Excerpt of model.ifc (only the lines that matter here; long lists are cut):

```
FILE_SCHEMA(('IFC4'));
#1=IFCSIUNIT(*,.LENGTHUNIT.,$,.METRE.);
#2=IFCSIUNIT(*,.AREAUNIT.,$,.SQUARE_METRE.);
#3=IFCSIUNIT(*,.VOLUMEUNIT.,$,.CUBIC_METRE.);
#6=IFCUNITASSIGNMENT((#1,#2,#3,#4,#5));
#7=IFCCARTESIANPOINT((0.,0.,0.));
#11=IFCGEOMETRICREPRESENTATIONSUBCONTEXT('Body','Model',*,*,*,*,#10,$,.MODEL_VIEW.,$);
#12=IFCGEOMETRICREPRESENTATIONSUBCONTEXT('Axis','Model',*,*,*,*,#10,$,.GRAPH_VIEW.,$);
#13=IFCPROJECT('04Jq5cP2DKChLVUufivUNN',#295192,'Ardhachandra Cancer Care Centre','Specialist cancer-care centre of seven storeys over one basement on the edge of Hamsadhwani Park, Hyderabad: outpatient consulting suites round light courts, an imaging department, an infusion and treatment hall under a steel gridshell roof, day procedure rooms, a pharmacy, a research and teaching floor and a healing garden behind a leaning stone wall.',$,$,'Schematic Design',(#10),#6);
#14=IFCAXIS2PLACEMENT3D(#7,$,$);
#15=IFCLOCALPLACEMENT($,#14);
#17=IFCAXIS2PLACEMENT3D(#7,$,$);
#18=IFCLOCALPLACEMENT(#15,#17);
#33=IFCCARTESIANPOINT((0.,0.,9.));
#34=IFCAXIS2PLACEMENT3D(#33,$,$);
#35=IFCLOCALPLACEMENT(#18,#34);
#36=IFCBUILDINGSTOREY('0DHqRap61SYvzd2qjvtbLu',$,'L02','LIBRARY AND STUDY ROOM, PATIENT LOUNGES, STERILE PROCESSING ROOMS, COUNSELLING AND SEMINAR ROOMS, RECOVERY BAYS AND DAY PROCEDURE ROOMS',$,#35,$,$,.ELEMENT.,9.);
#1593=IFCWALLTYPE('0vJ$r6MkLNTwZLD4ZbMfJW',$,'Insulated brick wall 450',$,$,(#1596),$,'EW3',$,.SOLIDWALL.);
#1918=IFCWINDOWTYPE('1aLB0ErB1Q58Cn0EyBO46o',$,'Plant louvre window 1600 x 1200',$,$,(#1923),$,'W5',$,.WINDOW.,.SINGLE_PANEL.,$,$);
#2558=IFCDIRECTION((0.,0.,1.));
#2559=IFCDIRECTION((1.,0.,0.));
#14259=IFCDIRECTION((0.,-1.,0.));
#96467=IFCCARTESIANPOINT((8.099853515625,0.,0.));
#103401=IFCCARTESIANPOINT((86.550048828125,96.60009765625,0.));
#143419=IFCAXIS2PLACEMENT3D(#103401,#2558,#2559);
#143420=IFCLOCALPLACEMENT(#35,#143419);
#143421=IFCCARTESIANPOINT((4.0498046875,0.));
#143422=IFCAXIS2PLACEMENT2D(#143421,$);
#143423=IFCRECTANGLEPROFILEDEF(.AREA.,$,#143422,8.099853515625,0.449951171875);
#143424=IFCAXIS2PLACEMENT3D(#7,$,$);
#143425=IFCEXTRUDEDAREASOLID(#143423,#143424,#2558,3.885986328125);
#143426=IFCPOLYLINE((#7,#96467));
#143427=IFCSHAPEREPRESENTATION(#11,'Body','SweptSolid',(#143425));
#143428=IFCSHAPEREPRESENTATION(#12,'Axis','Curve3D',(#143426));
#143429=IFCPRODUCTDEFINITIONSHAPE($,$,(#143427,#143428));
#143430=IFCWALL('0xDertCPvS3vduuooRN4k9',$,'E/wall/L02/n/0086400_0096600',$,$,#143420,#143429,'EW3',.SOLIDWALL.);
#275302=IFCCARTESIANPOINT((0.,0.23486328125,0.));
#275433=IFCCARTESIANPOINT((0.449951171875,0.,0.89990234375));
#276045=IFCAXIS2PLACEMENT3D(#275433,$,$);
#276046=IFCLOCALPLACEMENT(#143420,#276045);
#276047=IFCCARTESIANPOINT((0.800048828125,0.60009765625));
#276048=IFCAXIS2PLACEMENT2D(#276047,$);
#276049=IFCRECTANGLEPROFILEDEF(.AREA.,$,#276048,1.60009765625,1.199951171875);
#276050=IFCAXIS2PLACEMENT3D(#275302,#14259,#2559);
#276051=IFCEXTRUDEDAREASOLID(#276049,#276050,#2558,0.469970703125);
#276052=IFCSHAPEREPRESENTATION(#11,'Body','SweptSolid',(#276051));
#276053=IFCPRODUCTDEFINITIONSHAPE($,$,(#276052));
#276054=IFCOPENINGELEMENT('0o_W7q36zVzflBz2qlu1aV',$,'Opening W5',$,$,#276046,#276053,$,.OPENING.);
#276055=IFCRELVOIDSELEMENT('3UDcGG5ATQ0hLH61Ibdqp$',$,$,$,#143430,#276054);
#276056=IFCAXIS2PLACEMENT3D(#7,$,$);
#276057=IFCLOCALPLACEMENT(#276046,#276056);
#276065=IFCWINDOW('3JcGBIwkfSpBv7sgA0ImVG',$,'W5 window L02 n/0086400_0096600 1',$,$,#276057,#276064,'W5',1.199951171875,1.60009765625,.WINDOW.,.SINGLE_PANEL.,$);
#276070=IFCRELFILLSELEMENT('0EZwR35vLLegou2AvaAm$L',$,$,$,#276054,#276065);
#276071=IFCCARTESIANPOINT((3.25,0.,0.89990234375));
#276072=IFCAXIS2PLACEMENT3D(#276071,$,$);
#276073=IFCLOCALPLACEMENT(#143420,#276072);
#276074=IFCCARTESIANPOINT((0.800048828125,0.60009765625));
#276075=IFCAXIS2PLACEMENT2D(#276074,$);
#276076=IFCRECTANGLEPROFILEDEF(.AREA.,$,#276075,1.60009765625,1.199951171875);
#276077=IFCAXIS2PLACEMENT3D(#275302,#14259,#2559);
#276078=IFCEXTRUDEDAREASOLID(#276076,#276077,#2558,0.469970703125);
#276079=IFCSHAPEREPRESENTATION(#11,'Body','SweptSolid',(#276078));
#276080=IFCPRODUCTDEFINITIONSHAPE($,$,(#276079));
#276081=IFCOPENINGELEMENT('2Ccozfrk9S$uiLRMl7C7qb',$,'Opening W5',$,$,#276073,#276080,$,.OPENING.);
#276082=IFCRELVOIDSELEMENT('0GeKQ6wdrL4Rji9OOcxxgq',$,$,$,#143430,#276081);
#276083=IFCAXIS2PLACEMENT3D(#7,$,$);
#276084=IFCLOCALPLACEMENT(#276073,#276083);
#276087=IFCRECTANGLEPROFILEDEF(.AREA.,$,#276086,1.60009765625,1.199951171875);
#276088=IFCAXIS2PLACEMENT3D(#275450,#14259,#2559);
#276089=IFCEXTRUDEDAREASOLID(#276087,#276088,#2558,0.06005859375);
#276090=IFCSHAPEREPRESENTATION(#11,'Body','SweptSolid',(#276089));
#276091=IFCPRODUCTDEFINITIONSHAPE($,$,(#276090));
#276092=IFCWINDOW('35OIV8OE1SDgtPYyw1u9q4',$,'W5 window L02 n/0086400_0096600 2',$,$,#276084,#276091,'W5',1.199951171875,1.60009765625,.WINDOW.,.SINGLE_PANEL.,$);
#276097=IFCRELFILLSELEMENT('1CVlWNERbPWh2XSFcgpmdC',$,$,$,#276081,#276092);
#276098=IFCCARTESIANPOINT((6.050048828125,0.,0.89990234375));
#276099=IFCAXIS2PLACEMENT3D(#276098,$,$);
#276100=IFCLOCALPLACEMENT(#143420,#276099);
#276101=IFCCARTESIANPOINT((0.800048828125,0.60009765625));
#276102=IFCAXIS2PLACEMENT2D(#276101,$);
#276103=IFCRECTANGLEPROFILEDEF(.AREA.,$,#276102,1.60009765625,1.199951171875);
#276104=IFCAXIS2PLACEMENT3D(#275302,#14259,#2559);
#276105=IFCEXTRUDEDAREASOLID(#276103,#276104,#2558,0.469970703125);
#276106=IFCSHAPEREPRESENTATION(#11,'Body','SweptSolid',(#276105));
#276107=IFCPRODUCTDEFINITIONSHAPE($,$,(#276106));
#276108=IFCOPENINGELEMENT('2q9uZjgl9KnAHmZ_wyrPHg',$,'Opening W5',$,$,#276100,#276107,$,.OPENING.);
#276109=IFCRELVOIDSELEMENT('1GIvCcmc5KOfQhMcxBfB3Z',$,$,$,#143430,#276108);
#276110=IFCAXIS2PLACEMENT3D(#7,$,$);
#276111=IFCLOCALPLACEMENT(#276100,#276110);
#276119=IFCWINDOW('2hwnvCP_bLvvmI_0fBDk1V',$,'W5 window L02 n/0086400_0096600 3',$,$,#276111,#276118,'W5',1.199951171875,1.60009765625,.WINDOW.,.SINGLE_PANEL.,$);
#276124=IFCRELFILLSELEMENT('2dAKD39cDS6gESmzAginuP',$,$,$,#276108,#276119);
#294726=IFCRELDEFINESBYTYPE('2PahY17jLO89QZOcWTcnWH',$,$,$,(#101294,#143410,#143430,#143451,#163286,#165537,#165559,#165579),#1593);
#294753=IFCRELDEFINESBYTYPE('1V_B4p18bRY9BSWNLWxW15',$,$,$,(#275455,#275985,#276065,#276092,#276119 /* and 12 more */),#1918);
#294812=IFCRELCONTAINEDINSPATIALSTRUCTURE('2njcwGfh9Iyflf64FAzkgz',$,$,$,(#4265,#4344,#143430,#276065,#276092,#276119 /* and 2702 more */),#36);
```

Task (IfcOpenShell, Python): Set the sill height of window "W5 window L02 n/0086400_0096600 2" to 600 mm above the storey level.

```python
import numpy as np
import ifcopenshell
import ifcopenshell.api.geometry
import ifcopenshell.geom
import ifcopenshell.util.element
import ifcopenshell.util.placement
import ifcopenshell.util.shape
import ifcopenshell.util.unit

model = ifcopenshell.open("model.ifc")
unit_scale = ifcopenshell.util.unit.calculate_unit_scale(model)

window = model.by_guid("35OIV8OE1SDgtPYyw1u9q4")
opening = window.FillsVoids[0].RelatingOpeningElement
storey = ifcopenshell.util.element.get_container(window, ifc_class="IfcBuildingStorey")
level = ifcopenshell.util.placement.get_local_placement(storey.ObjectPlacement)[2, 3]

# The opening's origin need not be at the sill, so measure its lowest point.
shape = ifcopenshell.geom.create_shape(ifcopenshell.geom.settings(), opening)
bottom = ifcopenshell.util.shape.get_shape_bottom_elevation(shape, shape.geometry) / unit_scale
dz = level + 0.6 / unit_scale - bottom

shift = np.array([0.0, 0.0, dz])
# The window is placed relative to its opening, so it follows when the opening moves.
matrix = ifcopenshell.util.placement.get_local_placement(opening.ObjectPlacement)
matrix[:3, 3] += shift
ifcopenshell.api.geometry.edit_object_placement(
    model, product=opening, matrix=matrix, is_si=False, should_transform_children=True
)

print(f"moved by {dz * unit_scale:+.3f} m")

model.write("model_updated.ifc")
```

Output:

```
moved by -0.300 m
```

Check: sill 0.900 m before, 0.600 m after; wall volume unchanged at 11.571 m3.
